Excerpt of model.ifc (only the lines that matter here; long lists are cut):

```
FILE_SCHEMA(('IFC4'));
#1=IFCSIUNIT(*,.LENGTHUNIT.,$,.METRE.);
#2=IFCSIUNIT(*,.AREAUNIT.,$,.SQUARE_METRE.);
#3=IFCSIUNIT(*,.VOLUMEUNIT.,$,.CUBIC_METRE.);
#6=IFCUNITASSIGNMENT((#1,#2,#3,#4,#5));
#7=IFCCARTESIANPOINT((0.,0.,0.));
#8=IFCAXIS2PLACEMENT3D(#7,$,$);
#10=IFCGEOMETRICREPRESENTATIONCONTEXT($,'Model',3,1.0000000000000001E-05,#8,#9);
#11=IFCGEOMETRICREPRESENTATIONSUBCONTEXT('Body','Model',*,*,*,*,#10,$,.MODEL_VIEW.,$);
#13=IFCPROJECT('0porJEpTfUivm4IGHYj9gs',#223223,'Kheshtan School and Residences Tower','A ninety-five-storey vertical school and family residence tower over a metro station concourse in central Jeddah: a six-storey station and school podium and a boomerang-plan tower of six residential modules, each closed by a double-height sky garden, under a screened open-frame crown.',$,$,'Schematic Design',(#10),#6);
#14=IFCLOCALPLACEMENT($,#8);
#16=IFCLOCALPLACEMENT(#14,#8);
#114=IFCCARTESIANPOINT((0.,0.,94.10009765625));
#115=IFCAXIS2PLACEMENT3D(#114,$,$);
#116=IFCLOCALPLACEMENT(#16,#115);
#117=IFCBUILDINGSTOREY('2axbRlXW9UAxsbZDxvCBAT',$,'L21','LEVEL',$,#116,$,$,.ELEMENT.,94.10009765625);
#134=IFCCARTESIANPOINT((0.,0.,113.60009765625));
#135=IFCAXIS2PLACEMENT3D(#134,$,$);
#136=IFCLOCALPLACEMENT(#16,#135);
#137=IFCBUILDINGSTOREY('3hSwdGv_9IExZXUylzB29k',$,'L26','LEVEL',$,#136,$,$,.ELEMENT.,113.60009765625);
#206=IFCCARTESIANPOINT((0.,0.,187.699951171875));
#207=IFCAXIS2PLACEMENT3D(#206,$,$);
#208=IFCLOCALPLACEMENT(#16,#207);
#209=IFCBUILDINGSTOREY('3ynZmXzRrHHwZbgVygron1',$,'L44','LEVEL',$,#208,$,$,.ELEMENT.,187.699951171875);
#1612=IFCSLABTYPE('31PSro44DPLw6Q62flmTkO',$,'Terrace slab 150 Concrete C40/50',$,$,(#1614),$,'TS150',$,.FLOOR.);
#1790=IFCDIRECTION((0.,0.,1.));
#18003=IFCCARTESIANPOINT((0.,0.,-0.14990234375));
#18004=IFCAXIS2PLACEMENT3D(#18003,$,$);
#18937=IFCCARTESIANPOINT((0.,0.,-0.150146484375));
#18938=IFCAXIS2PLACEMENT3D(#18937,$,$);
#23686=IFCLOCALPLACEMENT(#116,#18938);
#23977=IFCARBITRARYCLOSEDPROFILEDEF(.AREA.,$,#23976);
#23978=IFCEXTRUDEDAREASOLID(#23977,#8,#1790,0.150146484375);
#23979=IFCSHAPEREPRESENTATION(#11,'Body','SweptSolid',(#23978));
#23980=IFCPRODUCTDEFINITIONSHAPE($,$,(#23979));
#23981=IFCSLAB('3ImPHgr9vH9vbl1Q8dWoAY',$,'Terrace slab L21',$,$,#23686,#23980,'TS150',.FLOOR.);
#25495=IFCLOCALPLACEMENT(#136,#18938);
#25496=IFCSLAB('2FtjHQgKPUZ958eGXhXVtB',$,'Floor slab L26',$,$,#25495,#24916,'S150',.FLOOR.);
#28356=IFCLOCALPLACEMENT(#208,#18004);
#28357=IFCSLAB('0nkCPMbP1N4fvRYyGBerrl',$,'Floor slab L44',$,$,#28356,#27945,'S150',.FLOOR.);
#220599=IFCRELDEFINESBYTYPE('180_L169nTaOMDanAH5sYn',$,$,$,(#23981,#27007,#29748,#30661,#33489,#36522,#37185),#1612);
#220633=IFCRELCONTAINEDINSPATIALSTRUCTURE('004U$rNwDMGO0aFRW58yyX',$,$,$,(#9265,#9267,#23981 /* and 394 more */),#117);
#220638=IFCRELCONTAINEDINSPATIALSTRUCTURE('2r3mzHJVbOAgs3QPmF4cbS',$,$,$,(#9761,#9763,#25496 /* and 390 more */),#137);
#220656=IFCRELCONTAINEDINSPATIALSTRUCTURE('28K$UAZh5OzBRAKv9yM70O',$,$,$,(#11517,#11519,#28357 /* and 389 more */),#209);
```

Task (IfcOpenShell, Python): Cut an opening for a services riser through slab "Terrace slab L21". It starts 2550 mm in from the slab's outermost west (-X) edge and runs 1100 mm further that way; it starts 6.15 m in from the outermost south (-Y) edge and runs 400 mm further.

```python
import numpy as np
import ifcopenshell
import ifcopenshell.api.feature
import ifcopenshell.api.geometry
import ifcopenshell.api.root
import ifcopenshell.geom
import ifcopenshell.util.placement
import ifcopenshell.util.representation
import ifcopenshell.util.shape
import ifcopenshell.util.unit

model = ifcopenshell.open("model.ifc")
unit_scale = ifcopenshell.util.unit.calculate_unit_scale(model)
settings = ifcopenshell.geom.settings()


def volume(element):
    """Net volume in cubic metres, openings subtracted."""
    shape = ifcopenshell.geom.create_shape(settings, element)
    return ifcopenshell.util.shape.get_volume(shape.geometry)


slab = model.by_id(23981)
before = volume(slab)

# Extent in the slab's own axes, in metres. The edges named are its -X and -Y sides.
slab_shape = ifcopenshell.geom.create_shape(settings, slab)
vertices = ifcopenshell.util.shape.get_vertices(slab_shape.geometry)
x_min, y_min, bottom = vertices.min(axis=0)
top = vertices[:, 2].max()

opening = ifcopenshell.api.root.create_entity(model, ifc_class="IfcOpeningElement", name="Services riser opening", predefined_type="OPENING")
context = ifcopenshell.util.representation.get_context(model, "Model", "Body", "MODEL_VIEW")
width, depth = 1.1, 0.4
outline = [(0.0, 0.0), (width, 0.0), (width, depth), (0.0, depth), (0.0, 0.0)]
# Overshoot both faces by 50 mm so the cut is clean.
shape = ifcopenshell.api.geometry.add_slab_representation(
    model, context=context, depth=top - bottom + 0.1, polyline=outline
)
ifcopenshell.api.geometry.assign_representation(model, product=opening, representation=shape)

matrix = ifcopenshell.util.placement.get_local_placement(slab.ObjectPlacement)
matrix[:, 3] = matrix @ np.append(np.array([x_min + 2.55, y_min + 6.15, bottom - 0.05]) / unit_scale, 1.0)
ifcopenshell.api.geometry.edit_object_placement(model, product=opening, matrix=matrix, is_si=False)
ifcopenshell.api.feature.add_feature(model, feature=opening, element=slab)

after = volume(slab)

print(f"slab volume {before:.3f} -> {after:.3f} m3")

model.write("model_updated.ifc")
```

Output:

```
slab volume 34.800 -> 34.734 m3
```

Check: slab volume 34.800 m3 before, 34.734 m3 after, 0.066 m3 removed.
